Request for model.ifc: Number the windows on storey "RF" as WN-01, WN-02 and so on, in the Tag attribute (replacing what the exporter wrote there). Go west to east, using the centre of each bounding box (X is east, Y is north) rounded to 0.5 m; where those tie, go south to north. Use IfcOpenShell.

First a look at what the model holds.

```python
import ifcopenshell
import ifcopenshell.util.element
import ifcopenshell.util.placement

model = ifcopenshell.open("model.ifc")
print(model.schema)
storey = next(s for s in model.by_type("IfcBuildingStorey") if s.Name == "RF")
windows = [e for e in ifcopenshell.util.element.get_decomposition(storey) if e.is_a("IfcWindow")]
for e in sorted(windows, key=lambda e: e.id()):
    origin = ifcopenshell.util.placement.get_local_placement(e.ObjectPlacement)[:3, 3]
    print(e.id(), e.Tag, e.Name, origin.round(2) + 0.0, sep=" | ")
```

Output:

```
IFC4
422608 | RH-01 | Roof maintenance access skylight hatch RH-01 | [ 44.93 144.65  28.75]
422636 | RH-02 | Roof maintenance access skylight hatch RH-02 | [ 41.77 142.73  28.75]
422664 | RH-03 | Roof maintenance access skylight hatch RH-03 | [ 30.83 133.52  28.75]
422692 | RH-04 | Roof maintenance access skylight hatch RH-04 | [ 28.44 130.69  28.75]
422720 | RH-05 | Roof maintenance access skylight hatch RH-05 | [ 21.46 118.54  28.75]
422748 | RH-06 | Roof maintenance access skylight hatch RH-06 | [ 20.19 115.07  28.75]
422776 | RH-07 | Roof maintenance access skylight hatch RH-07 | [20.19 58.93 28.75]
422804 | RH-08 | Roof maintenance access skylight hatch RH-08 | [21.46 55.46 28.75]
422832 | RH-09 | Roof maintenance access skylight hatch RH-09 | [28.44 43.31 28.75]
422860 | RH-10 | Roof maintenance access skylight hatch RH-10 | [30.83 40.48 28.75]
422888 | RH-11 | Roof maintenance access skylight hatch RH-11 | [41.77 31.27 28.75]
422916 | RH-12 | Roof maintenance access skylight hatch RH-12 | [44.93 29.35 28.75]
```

```python
import ifcopenshell
import ifcopenshell.geom
import ifcopenshell.util.element
import ifcopenshell.util.shape

model = ifcopenshell.open("model.ifc")
settings = ifcopenshell.geom.settings()
settings.set("use-world-coords", True)


def centre(element):
    shape = ifcopenshell.geom.create_shape(settings, element)
    return ifcopenshell.util.shape.get_bbox_centroid(shape.geometry)


storey = next(s for s in model.by_type("IfcBuildingStorey") if s.Name == "RF")
windows = [e for e in ifcopenshell.util.element.get_decomposition(storey) if e.is_a("IfcWindow")]

# Insertion points can sit at a corner or the storey origin, so sort by the geometry (in metres).
centres = {e: centre(e) for e in windows}
windows.sort(key=lambda e: (round(centres[e][0] / 0.5), centres[e][1]))

for i, e in enumerate(windows, start=1):
    number = f"WN-{i:02d}"
    e.Tag = number
    print(e.id(), number)

model.write("model_edited.ifc")
```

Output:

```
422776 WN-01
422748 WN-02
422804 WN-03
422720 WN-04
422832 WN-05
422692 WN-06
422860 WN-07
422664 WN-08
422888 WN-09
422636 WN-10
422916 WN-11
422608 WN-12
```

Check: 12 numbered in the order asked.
